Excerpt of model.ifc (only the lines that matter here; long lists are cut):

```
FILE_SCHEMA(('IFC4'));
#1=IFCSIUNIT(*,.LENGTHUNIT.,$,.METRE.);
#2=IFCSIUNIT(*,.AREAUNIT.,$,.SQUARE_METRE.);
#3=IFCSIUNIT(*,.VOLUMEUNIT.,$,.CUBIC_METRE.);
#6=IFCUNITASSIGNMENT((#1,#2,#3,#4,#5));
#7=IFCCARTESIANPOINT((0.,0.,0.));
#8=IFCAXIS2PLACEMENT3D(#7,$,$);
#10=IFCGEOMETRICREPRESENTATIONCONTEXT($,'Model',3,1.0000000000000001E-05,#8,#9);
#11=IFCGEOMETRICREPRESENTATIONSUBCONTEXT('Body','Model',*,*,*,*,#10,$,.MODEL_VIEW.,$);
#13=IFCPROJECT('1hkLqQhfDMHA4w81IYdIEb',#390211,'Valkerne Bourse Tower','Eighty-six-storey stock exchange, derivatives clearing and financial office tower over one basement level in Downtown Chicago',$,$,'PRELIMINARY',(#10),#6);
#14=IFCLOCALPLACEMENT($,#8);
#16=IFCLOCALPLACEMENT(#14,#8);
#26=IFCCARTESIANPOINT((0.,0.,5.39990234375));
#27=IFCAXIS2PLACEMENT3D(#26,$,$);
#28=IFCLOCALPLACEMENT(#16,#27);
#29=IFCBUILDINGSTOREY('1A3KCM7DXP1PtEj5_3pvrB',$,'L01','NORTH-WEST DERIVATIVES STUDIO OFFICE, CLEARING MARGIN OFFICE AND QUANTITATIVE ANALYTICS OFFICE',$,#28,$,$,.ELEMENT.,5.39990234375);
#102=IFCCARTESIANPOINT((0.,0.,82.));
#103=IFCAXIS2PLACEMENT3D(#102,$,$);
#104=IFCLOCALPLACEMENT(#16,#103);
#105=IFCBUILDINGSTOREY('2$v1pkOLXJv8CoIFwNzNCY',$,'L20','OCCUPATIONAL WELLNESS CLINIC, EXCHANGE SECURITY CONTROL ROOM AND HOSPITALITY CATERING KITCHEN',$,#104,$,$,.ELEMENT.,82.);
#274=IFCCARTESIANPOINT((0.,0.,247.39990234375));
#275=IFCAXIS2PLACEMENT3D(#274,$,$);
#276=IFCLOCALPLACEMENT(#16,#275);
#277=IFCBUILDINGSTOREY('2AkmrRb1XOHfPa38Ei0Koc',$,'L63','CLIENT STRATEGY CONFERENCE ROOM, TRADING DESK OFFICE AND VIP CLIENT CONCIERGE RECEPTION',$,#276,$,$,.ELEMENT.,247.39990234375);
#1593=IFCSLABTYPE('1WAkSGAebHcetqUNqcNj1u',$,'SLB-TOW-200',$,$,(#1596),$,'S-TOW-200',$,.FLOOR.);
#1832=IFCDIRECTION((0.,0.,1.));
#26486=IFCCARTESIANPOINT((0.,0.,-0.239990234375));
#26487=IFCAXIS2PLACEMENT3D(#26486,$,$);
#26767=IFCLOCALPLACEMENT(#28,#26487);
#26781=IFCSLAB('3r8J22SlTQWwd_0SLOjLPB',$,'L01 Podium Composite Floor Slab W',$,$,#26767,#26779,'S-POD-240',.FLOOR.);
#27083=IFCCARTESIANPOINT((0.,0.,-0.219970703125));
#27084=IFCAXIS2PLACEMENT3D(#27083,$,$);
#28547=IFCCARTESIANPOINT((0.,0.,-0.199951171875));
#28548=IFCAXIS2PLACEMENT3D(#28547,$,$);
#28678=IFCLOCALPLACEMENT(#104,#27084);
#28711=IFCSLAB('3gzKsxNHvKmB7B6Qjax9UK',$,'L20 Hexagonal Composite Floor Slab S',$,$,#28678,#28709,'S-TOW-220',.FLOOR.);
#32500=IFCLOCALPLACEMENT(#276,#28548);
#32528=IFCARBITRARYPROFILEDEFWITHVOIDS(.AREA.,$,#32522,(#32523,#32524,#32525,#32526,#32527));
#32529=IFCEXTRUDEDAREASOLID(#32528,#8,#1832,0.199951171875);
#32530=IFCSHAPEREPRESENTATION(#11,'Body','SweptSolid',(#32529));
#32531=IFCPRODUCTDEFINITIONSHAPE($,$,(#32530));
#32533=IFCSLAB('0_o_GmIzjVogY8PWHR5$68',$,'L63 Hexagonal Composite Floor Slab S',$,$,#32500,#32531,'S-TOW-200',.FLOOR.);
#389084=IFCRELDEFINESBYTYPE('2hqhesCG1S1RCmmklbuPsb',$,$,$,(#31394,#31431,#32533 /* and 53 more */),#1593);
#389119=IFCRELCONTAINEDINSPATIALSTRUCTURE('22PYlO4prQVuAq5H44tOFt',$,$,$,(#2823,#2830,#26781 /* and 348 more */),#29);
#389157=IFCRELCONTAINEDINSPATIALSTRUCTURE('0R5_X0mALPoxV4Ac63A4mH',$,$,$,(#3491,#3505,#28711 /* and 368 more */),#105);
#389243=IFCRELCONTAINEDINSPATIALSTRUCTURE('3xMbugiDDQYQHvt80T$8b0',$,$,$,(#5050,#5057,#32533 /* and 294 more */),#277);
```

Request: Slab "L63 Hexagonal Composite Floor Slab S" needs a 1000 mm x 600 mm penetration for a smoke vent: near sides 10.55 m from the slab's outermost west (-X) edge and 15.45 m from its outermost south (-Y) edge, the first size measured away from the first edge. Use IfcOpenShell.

```python
import numpy as np
import ifcopenshell
import ifcopenshell.api.feature
import ifcopenshell.api.geometry
import ifcopenshell.api.root
import ifcopenshell.geom
import ifcopenshell.util.placement
import ifcopenshell.util.representation
import ifcopenshell.util.shape
import ifcopenshell.util.unit

model = ifcopenshell.open("model.ifc")
unit_scale = ifcopenshell.util.unit.calculate_unit_scale(model)
settings = ifcopenshell.geom.settings()


def volume(element):
    """Net volume in cubic metres, openings subtracted."""
    shape = ifcopenshell.geom.create_shape(settings, element)
    return ifcopenshell.util.shape.get_volume(shape.geometry)


slab = model.by_id(32533)
before = volume(slab)

# Extent in the slab's own axes, in metres. The edges named are its -X and -Y sides.
slab_shape = ifcopenshell.geom.create_shape(settings, slab)
vertices = ifcopenshell.util.shape.get_vertices(slab_shape.geometry)
x_min, y_min, bottom = vertices.min(axis=0)
top = vertices[:, 2].max()

opening = ifcopenshell.api.root.create_entity(model, ifc_class="IfcOpeningElement", name="Smoke vent opening", predefined_type="OPENING")
context = ifcopenshell.util.representation.get_context(model, "Model", "Body", "MODEL_VIEW")
width, depth = 1, 0.6
outline = [(0.0, 0.0), (width, 0.0), (width, depth), (0.0, depth), (0.0, 0.0)]
# Overshoot both faces by 50 mm so the cut is clean.
shape = ifcopenshell.api.geometry.add_slab_representation(
    model, context=context, depth=top - bottom + 0.1, polyline=outline
)
ifcopenshell.api.geometry.assign_representation(model, product=opening, representation=shape)

matrix = ifcopenshell.util.placement.get_local_placement(slab.ObjectPlacement)
matrix[:, 3] = matrix @ np.append(np.array([x_min + 10.55, y_min + 15.45, bottom - 0.05]) / unit_scale, 1.0)
ifcopenshell.api.geometry.edit_object_placement(model, product=opening, matrix=matrix, is_si=False)
ifcopenshell.api.feature.add_feature(model, feature=opening, element=slab)

after = volume(slab)

print(f"slab volume {before:.3f} -> {after:.3f} m3")

model.write("model_v2.ifc")
```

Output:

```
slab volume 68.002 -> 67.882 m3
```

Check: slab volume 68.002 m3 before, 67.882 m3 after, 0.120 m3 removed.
